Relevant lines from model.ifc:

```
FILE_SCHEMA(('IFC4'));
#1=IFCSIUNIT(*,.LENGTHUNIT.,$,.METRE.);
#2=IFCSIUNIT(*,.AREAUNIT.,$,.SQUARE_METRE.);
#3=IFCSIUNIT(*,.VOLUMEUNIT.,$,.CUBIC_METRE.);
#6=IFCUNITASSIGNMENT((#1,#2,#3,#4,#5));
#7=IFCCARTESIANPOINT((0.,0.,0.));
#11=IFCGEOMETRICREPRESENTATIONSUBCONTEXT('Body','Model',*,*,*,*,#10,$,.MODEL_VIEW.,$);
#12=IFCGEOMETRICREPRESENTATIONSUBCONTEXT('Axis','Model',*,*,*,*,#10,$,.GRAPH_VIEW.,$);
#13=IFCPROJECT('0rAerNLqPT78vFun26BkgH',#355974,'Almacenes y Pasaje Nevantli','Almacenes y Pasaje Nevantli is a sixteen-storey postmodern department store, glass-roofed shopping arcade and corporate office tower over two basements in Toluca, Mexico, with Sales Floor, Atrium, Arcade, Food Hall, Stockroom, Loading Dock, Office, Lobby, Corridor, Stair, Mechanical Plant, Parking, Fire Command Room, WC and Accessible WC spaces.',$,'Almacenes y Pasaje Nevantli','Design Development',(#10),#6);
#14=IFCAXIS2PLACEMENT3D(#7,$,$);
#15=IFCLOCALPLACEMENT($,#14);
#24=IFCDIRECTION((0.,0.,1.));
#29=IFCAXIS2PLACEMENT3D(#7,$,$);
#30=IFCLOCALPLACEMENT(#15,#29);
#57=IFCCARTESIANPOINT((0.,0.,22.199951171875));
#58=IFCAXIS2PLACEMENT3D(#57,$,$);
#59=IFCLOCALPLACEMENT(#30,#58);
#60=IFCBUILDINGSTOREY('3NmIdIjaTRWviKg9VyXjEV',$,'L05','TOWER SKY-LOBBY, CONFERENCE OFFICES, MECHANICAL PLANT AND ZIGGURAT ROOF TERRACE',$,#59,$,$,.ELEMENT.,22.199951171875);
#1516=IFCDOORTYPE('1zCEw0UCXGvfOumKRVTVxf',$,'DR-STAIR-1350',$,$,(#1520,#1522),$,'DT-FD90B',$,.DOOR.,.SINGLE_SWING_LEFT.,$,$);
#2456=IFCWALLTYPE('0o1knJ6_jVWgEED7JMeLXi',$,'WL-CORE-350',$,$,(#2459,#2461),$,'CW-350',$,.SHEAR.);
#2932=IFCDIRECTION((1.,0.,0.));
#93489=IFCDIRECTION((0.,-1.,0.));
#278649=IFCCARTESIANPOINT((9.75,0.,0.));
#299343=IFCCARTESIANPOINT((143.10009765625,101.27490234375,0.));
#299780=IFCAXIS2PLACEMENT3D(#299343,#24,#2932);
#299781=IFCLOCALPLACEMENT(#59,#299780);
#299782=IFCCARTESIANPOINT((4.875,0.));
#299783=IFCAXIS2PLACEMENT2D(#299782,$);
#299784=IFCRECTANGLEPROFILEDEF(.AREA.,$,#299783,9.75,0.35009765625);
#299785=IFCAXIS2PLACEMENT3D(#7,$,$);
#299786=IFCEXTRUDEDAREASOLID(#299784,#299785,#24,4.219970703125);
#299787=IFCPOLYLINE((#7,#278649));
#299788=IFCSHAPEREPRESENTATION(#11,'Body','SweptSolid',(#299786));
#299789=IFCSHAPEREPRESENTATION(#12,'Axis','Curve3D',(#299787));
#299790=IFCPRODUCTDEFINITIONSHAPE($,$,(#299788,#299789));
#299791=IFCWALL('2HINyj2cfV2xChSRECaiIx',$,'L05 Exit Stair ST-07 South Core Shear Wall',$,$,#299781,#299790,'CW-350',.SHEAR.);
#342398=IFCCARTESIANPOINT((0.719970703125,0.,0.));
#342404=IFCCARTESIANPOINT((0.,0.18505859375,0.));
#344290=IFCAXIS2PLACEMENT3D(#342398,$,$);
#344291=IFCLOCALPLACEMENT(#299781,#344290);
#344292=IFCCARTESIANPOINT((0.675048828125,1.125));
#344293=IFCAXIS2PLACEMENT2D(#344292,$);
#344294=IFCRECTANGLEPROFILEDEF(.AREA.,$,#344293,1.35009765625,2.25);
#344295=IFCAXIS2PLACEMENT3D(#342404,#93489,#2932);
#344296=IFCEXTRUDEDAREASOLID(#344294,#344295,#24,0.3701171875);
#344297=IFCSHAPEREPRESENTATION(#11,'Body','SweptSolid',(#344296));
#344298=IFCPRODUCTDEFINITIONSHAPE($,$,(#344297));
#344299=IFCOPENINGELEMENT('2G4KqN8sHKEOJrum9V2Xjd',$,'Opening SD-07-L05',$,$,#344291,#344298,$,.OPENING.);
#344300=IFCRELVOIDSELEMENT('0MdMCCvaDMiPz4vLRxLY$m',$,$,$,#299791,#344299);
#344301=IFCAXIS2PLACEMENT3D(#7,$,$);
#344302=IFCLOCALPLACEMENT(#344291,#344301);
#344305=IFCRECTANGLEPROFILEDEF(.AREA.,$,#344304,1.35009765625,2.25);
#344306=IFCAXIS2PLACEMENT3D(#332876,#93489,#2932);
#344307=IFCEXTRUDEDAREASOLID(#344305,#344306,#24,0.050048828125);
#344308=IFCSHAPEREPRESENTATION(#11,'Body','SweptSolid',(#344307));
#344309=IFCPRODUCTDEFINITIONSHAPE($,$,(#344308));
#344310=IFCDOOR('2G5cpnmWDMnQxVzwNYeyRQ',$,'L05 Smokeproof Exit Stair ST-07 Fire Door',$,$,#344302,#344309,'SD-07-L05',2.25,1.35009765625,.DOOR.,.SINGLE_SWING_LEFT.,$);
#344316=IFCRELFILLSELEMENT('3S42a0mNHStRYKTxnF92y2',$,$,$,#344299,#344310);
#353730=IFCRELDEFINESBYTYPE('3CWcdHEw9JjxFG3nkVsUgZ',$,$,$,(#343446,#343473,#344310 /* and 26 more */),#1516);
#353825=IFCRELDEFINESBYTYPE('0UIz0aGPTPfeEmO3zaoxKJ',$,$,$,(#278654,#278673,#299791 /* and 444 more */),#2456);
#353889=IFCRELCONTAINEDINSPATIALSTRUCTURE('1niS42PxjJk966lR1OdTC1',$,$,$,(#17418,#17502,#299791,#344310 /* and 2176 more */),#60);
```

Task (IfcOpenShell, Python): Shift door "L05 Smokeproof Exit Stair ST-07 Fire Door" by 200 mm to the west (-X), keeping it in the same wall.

```python
import ifcopenshell
import ifcopenshell.api.geometry
import ifcopenshell.util.placement
import ifcopenshell.util.unit

model = ifcopenshell.open("model.ifc")
unit_scale = ifcopenshell.util.unit.calculate_unit_scale(model)

door = model.by_guid("2G5cpnmWDMnQxVzwNYeyRQ")
opening = door.FillsVoids[0].RelatingOpeningElement
wall = opening.VoidsElements[0].RelatingBuildingElement

wall_matrix = ifcopenshell.util.placement.get_local_placement(wall.ObjectPlacement)
shift = wall_matrix[:3, 0] * -0.2 / unit_scale
before = ifcopenshell.util.placement.get_local_placement(door.ObjectPlacement)[:3, 3].copy()

# The door is placed relative to its opening, so it follows when the opening moves.
matrix = ifcopenshell.util.placement.get_local_placement(opening.ObjectPlacement)
matrix[:3, 3] += shift
ifcopenshell.api.geometry.edit_object_placement(
    model, product=opening, matrix=matrix, is_si=False, should_transform_children=True
)

after = ifcopenshell.util.placement.get_local_placement(door.ObjectPlacement)[:3, 3]
print("door moved by", (after - before).round(3) + 0.0)

model.write("model_v2.ifc")
```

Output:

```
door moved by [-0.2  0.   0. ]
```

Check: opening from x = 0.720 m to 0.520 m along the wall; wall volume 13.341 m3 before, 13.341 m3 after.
